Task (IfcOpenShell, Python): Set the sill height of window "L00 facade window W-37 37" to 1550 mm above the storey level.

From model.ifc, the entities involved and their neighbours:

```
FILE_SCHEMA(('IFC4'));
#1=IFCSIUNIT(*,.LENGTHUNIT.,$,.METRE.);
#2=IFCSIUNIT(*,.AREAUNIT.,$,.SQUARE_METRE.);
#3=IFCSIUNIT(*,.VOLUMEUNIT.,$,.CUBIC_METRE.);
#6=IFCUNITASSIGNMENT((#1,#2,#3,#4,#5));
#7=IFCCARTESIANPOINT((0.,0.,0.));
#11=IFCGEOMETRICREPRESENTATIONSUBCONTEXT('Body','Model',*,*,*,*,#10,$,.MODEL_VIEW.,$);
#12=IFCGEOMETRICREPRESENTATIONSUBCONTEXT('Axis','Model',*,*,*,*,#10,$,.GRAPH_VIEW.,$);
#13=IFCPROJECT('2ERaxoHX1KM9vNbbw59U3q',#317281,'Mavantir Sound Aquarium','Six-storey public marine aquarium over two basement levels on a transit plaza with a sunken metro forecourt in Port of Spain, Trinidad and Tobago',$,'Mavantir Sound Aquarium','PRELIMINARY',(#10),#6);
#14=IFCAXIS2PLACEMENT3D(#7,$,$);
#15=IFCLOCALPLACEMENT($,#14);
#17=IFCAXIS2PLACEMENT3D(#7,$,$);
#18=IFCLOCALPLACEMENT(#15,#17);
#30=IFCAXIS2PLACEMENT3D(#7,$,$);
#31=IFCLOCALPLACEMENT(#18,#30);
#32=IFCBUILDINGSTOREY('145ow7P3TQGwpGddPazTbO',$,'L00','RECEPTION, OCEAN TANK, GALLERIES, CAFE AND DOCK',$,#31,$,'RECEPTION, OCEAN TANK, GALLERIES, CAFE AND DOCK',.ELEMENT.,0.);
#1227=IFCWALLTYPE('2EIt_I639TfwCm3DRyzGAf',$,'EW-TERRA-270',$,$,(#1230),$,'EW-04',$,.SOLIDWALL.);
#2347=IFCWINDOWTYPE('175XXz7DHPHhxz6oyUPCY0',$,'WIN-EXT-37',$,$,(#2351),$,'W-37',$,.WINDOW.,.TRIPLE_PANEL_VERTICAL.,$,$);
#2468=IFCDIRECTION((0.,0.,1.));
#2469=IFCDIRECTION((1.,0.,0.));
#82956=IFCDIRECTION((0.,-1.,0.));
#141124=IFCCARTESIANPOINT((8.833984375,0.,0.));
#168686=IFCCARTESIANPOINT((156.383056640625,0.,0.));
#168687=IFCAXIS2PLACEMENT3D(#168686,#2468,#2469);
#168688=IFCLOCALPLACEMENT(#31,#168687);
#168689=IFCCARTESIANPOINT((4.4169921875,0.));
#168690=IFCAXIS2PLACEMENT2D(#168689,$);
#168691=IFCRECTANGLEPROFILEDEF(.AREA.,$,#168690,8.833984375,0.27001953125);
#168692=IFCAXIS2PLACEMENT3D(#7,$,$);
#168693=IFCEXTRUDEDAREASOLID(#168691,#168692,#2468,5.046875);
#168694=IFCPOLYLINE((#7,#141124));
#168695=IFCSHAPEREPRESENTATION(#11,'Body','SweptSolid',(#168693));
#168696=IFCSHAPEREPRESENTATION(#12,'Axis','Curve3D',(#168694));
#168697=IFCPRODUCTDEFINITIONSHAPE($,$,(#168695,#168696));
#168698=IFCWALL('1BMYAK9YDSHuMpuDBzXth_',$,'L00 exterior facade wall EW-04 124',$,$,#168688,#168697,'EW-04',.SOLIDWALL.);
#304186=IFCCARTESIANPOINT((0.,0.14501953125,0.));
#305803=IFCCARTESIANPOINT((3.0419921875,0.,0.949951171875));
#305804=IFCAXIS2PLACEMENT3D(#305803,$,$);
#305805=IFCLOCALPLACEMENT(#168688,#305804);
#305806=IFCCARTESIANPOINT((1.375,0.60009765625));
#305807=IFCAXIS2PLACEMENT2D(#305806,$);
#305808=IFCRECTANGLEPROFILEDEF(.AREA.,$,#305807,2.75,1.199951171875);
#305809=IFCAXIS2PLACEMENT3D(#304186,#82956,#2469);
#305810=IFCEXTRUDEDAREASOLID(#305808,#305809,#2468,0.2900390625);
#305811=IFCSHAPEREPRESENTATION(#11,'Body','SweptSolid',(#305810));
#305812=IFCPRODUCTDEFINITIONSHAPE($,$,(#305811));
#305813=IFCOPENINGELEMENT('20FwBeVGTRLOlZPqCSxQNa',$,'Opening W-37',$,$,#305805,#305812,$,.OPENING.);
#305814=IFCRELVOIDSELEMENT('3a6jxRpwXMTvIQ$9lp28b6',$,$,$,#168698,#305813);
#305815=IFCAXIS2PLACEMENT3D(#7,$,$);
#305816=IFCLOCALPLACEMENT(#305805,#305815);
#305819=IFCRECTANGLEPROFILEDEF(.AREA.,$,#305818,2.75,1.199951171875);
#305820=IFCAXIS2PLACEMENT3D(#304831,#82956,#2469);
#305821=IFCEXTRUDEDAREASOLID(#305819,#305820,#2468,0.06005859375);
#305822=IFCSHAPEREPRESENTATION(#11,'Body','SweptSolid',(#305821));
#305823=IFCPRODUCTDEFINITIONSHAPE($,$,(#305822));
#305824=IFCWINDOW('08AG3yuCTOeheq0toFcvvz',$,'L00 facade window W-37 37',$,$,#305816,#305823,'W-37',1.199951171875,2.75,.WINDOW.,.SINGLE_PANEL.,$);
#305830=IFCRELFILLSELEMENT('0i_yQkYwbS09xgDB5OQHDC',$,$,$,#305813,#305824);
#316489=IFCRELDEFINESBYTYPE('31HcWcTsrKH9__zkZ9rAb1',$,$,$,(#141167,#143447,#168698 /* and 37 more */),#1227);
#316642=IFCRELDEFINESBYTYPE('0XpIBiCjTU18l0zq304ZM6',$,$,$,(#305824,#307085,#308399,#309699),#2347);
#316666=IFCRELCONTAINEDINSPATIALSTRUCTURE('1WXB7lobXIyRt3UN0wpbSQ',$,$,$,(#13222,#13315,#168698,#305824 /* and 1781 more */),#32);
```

```python
import numpy as np
import ifcopenshell
import ifcopenshell.api.geometry
import ifcopenshell.geom
import ifcopenshell.util.element
import ifcopenshell.util.placement
import ifcopenshell.util.shape
import ifcopenshell.util.unit

model = ifcopenshell.open("model.ifc")
unit_scale = ifcopenshell.util.unit.calculate_unit_scale(model)

window = model.by_guid("08AG3yuCTOeheq0toFcvvz")
opening = window.FillsVoids[0].RelatingOpeningElement
storey = ifcopenshell.util.element.get_container(window, ifc_class="IfcBuildingStorey")
level = ifcopenshell.util.placement.get_local_placement(storey.ObjectPlacement)[2, 3]

# The opening's origin need not be at the sill, so measure its lowest point.
shape = ifcopenshell.geom.create_shape(ifcopenshell.geom.settings(), opening)
bottom = ifcopenshell.util.shape.get_shape_bottom_elevation(shape, shape.geometry) / unit_scale
dz = level + 1.55 - bottom

shift = np.array([0.0, 0.0, dz])
# The window is placed relative to its opening, so it follows when the opening moves.
matrix = ifcopenshell.util.placement.get_local_placement(opening.ObjectPlacement)
matrix[:3, 3] += shift
ifcopenshell.api.geometry.edit_object_placement(
    model, product=opening, matrix=matrix, is_si=False, should_transform_children=True
)

print(f"moved by {dz * unit_scale:+.3f} m")

model.write("model_updated.ifc")
```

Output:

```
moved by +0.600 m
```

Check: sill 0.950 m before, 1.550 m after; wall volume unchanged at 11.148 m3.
